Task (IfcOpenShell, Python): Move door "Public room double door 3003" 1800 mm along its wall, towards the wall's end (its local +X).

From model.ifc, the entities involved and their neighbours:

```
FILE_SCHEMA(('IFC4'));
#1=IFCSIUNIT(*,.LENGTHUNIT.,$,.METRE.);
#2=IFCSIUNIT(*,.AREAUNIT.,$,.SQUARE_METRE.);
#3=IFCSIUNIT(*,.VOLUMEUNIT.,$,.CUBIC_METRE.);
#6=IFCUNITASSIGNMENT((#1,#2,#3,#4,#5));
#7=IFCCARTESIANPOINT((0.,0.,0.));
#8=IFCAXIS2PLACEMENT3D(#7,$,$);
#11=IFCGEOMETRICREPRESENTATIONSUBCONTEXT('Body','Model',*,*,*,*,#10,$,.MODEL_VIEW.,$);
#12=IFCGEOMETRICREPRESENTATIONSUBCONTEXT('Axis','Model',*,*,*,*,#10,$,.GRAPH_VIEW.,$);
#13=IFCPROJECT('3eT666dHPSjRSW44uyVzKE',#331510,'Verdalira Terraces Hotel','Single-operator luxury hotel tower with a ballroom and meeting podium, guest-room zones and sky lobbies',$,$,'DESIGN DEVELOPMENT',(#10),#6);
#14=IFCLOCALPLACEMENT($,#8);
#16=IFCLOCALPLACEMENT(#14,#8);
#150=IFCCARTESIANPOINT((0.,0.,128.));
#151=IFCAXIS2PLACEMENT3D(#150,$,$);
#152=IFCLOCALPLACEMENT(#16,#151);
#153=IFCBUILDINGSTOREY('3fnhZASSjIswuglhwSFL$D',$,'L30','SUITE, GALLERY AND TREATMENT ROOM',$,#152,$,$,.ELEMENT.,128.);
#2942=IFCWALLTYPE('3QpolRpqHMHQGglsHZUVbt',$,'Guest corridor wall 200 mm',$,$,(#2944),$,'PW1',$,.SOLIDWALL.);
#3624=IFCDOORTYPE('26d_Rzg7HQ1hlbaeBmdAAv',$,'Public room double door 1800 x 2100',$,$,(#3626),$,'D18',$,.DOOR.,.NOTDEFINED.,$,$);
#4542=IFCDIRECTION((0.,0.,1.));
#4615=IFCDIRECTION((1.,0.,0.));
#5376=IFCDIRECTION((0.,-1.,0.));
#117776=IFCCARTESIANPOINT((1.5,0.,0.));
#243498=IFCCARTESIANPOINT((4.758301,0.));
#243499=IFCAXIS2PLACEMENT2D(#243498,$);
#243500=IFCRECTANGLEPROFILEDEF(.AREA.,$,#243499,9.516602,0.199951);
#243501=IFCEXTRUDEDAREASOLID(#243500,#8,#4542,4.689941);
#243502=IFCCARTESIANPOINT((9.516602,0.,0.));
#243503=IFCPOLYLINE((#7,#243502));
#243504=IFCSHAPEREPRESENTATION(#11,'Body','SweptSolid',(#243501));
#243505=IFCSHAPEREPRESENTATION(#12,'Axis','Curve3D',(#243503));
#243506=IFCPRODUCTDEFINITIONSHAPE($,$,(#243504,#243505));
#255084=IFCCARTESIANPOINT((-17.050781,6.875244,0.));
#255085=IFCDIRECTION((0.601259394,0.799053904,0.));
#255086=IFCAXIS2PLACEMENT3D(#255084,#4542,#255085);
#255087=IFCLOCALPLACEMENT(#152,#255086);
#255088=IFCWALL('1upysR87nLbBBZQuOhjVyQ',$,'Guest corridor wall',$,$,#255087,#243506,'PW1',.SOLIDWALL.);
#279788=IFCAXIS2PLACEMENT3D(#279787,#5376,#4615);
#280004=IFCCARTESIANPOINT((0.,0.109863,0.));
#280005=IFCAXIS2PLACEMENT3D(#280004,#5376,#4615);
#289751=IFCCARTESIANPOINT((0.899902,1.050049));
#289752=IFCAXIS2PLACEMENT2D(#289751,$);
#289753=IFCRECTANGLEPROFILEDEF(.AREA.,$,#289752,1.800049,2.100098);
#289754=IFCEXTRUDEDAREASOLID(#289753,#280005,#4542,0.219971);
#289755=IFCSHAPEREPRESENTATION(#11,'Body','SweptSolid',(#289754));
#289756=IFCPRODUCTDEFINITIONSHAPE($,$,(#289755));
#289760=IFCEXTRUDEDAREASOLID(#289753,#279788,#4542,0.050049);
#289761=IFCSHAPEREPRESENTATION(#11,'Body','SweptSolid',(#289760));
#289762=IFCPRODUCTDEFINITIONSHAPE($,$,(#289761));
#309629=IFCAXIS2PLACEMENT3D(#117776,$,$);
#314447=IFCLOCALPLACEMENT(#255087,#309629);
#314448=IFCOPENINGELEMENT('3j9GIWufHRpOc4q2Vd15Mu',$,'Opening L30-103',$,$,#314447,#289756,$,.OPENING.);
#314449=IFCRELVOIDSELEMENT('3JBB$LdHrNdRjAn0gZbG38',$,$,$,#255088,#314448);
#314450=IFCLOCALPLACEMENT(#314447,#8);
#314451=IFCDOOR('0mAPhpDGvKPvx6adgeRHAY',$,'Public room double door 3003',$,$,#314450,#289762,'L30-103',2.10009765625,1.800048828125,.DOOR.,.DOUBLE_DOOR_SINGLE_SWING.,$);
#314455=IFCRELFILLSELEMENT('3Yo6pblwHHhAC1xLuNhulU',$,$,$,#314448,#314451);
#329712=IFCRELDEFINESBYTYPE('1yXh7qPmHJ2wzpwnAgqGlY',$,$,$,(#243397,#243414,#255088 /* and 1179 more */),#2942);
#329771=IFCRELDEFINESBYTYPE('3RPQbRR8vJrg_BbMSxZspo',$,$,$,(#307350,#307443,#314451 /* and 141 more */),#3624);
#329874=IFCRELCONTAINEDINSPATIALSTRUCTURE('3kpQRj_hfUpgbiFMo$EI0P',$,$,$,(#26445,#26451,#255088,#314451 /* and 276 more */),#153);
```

```python
import ifcopenshell
import ifcopenshell.api.geometry
import ifcopenshell.util.placement
import ifcopenshell.util.unit

model = ifcopenshell.open("model.ifc")
unit_scale = ifcopenshell.util.unit.calculate_unit_scale(model)

door = model.by_guid("0mAPhpDGvKPvx6adgeRHAY")
opening = door.FillsVoids[0].RelatingOpeningElement
wall = opening.VoidsElements[0].RelatingBuildingElement

wall_matrix = ifcopenshell.util.placement.get_local_placement(wall.ObjectPlacement)
shift = wall_matrix[:3, 0] * 1.8 / unit_scale
before = ifcopenshell.util.placement.get_local_placement(door.ObjectPlacement)[:3, 3].copy()

# The door is placed relative to its opening, so it follows when the opening moves.
matrix = ifcopenshell.util.placement.get_local_placement(opening.ObjectPlacement)
matrix[:3, 3] += shift
ifcopenshell.api.geometry.edit_object_placement(
    model, product=opening, matrix=matrix, is_si=False, should_transform_children=True
)

after = ifcopenshell.util.placement.get_local_placement(door.ObjectPlacement)[:3, 3]
print("door moved by", (after - before).round(3) + 0.0)

model.write("model-out.ifc")
```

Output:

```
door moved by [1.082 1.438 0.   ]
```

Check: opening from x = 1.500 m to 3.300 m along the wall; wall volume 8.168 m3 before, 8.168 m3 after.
